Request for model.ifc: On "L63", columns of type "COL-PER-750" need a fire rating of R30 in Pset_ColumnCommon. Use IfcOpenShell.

First a look at what the model holds.

```python
import ifcopenshell
import ifcopenshell.util.element

model = ifcopenshell.open("model.ifc")
print(model.schema)
storey = next(s for s in model.by_type("IfcBuildingStorey") if s.Name == "L63")
columns = [e for e in ifcopenshell.util.element.get_decomposition(storey) if e.is_a("IfcColumn")]
seen = {}
for e in columns:
    element_type = ifcopenshell.util.element.get_type(e)
    key = (element_type.Name if element_type != e and element_type else None, ifcopenshell.util.element.get_pset(e, "Pset_ColumnCommon", "FireRating"))
    seen[key] = seen.get(key, 0) + 1
for (name, value), count in sorted(seen.items(), key=str):
    print(count, "x", name, "|", value)
```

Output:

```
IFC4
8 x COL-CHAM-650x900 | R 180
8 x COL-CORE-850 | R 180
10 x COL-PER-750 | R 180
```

```python
import ifcopenshell
import ifcopenshell.api.pset
import ifcopenshell.util.element

model = ifcopenshell.open("model.ifc")

storey = next(s for s in model.by_type("IfcBuildingStorey") if s.Name == "L63")
columns = [e for e in ifcopenshell.util.element.get_decomposition(storey) if e.is_a("IfcColumn")]

count = 0
for e in columns:
    element_type = ifcopenshell.util.element.get_type(e)
    if element_type in (None, e) or element_type.Name != "COL-PER-750":
        continue
    # add_pset returns the element's existing set when there is one.
    pset = ifcopenshell.api.pset.add_pset(model, product=e, name="Pset_ColumnCommon")
    ifcopenshell.api.pset.edit_pset(model, pset=pset, properties={"FireRating": "R30"})
    count += 1

print(count, "columns updated")

model.write("model_edited.ifc")
```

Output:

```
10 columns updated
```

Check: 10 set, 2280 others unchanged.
